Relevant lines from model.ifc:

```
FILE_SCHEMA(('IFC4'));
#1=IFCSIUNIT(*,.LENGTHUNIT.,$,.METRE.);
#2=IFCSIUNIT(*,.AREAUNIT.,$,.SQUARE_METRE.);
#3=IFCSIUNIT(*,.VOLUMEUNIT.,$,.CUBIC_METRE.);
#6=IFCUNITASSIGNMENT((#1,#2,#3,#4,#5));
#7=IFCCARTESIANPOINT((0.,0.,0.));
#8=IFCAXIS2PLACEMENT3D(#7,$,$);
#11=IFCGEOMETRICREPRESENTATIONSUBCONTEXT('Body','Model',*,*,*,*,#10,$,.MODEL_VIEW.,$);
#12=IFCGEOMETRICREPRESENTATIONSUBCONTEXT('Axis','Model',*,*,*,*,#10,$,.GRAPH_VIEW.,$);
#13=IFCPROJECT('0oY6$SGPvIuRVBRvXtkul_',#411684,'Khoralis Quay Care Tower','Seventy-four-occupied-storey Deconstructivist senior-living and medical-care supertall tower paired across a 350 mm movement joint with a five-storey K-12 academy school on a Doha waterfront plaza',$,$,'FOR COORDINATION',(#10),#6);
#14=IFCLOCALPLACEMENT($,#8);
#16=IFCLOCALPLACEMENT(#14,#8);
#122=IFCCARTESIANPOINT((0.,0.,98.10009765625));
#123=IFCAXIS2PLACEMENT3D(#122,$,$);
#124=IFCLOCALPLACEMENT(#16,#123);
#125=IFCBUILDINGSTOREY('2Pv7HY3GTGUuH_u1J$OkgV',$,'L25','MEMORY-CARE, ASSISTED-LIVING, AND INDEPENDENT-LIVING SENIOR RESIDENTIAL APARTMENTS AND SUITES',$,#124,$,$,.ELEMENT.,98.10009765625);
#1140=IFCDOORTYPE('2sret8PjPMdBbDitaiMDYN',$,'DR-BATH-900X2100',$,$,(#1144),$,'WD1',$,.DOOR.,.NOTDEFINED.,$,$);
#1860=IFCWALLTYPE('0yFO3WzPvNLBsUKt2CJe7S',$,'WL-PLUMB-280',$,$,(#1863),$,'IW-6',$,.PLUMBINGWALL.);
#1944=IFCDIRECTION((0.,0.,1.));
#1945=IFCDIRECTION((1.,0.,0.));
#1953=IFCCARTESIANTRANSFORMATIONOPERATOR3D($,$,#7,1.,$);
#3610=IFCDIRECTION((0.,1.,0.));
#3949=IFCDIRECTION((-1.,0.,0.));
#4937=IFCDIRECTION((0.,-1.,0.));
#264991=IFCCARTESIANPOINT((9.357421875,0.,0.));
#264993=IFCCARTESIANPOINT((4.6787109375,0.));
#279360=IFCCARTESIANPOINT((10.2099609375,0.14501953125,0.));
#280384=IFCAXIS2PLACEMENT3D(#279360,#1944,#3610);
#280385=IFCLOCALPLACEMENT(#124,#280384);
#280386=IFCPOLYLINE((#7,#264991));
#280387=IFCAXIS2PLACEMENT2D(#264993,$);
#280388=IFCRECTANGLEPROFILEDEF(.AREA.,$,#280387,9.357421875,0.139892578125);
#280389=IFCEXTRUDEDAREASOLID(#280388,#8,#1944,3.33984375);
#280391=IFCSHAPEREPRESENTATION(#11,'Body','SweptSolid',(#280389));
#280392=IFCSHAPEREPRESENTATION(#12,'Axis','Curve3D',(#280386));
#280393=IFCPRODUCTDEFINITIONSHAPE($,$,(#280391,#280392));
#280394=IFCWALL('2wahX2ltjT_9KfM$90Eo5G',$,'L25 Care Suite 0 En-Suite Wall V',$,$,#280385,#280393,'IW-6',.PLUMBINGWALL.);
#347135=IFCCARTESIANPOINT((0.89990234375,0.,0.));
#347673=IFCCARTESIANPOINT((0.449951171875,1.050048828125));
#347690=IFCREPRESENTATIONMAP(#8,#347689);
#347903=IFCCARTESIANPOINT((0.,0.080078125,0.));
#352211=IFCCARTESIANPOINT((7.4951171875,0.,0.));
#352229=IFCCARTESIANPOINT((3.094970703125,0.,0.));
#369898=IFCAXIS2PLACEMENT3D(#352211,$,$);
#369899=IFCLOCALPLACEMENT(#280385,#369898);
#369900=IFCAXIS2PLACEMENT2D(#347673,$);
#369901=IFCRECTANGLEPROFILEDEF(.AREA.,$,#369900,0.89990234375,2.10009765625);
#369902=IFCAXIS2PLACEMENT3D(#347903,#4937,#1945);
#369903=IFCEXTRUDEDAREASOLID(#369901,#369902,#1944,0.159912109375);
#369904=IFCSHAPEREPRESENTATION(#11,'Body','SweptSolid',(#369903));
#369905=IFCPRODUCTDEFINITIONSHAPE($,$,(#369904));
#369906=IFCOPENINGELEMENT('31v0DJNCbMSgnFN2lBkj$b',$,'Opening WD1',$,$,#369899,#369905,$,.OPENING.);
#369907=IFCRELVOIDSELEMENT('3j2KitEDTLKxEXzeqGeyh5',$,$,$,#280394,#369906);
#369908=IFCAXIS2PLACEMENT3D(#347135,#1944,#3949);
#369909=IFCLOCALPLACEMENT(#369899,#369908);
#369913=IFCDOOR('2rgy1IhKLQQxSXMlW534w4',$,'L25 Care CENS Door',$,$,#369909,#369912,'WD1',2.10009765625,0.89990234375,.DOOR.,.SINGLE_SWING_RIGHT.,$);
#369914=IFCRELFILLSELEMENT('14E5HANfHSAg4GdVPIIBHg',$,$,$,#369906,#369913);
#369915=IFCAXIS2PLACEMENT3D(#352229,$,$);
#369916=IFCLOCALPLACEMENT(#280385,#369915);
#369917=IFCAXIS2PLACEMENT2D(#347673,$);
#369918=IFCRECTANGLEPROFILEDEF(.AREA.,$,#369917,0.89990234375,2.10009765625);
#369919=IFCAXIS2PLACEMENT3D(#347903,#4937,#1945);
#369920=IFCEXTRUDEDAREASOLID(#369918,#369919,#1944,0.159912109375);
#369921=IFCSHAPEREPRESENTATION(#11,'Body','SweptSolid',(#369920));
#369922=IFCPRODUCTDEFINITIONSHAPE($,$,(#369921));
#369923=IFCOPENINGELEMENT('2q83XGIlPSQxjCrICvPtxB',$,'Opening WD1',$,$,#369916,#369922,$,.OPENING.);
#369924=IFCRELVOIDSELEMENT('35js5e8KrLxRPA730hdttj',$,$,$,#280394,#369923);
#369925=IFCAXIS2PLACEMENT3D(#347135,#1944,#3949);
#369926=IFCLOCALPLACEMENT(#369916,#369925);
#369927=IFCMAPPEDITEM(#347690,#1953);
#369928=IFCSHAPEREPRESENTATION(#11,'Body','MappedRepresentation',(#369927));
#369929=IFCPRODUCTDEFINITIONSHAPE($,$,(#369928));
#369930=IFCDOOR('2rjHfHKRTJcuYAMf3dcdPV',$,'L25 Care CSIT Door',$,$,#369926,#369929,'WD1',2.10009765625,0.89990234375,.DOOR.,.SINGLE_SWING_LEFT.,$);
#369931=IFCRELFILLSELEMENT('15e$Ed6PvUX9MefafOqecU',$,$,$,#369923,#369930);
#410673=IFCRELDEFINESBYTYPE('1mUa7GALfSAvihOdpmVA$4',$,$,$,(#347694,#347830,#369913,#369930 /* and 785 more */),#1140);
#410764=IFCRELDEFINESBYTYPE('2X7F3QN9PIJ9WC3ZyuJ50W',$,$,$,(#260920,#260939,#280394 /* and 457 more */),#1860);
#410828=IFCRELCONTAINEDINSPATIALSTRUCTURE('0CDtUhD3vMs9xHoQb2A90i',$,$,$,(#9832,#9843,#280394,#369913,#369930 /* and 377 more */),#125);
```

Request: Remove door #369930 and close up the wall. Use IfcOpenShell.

```python
import ifcopenshell
import ifcopenshell.api.feature
import ifcopenshell.api.root
import ifcopenshell.geom
import ifcopenshell.util.shape

model = ifcopenshell.open("model.ifc")
settings = ifcopenshell.geom.settings()


def volume(element):
    """Net volume in cubic metres, openings subtracted."""
    shape = ifcopenshell.geom.create_shape(settings, element)
    return ifcopenshell.util.shape.get_volume(shape.geometry)


door = model.by_guid("2rjHfHKRTJcuYAMf3dcdPV")
opening = door.FillsVoids[0].RelatingOpeningElement
wall = opening.VoidsElements[0].RelatingBuildingElement
before = volume(wall)

ifcopenshell.api.root.remove_product(model, product=door)
ifcopenshell.api.feature.remove_feature(model, feature=opening)

after = volume(wall)

print(f"wall volume {before:.3f} -> {after:.3f} m3")

model.write("model-out.ifc")
```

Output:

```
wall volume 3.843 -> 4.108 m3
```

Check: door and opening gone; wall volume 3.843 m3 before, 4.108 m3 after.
